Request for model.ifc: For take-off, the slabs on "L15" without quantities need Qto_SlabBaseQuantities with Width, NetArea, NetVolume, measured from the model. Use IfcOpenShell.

First a look at what the model holds.

```python
import ifcopenshell
import ifcopenshell.util.element
import ifcopenshell.util.unit

model = ifcopenshell.open("model.ifc")
print(model.schema)
for unit_type in ("LENGTHUNIT", "AREAUNIT", "VOLUMEUNIT"):
    print(unit_type, ifcopenshell.util.unit.calculate_unit_scale(model, unit_type))
storey = next(s for s in model.by_type("IfcBuildingStorey") if s.Name == "L15")
slabs = [e for e in ifcopenshell.util.element.get_decomposition(storey) if e.is_a("IfcSlab")]
for e in sorted(slabs, key=lambda e: e.id()):
    print(e.id(), e.is_a(), e.Name, list(ifcopenshell.util.element.get_psets(e, qtos_only=True)), sep=" | ")
```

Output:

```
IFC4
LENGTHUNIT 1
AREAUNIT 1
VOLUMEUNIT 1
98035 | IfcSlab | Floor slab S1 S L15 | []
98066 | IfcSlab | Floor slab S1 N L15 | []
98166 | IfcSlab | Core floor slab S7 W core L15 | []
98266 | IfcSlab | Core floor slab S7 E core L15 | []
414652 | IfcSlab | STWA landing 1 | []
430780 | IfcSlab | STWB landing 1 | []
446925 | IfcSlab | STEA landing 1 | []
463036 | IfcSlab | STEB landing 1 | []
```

```python
import ifcopenshell
import ifcopenshell.api.pset
import ifcopenshell.geom
import ifcopenshell.util.element
import ifcopenshell.util.shape
import ifcopenshell.util.unit

model = ifcopenshell.open("model.ifc")
unit_scale = ifcopenshell.util.unit.calculate_unit_scale(model)
area_scale = ifcopenshell.util.unit.calculate_unit_scale(model, "AREAUNIT")
volume_scale = ifcopenshell.util.unit.calculate_unit_scale(model, "VOLUMEUNIT")
settings = ifcopenshell.geom.settings()

storey = next(s for s in model.by_type("IfcBuildingStorey") if s.Name == "L15")
slabs = [e for e in ifcopenshell.util.element.get_decomposition(storey) if e.is_a("IfcSlab")]

for e in sorted(slabs, key=lambda e: e.id()):
    if ifcopenshell.util.element.get_psets(e, qtos_only=True, should_inherit=False):
        continue
    # Geometry comes back in metres, in the element's own axes.
    shape = ifcopenshell.geom.create_shape(settings, e)
    values = {
        "Width": ifcopenshell.util.shape.get_z(shape.geometry) / unit_scale,
        "NetArea": ifcopenshell.util.shape.get_footprint_area(shape.geometry) / area_scale,
        "NetVolume": ifcopenshell.util.shape.get_volume(shape.geometry) / volume_scale,
    }
    qto = ifcopenshell.api.pset.add_qto(model, product=e, name="Qto_SlabBaseQuantities")
    ifcopenshell.api.pset.edit_qto(model, qto=qto, properties=values)
    print(e.id(), {k: round(v, 3) for k, v in values.items()})

model.write("model_edited.ifc")
```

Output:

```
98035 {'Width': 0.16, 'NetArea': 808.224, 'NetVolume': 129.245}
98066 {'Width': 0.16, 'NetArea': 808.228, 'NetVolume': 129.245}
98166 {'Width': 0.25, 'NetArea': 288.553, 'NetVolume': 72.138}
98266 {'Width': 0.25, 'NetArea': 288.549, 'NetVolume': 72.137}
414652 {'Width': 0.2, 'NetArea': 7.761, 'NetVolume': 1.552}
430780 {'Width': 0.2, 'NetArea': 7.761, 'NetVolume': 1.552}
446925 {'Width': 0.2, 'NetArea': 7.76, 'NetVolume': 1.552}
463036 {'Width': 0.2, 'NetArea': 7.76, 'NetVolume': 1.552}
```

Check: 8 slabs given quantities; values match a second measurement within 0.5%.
